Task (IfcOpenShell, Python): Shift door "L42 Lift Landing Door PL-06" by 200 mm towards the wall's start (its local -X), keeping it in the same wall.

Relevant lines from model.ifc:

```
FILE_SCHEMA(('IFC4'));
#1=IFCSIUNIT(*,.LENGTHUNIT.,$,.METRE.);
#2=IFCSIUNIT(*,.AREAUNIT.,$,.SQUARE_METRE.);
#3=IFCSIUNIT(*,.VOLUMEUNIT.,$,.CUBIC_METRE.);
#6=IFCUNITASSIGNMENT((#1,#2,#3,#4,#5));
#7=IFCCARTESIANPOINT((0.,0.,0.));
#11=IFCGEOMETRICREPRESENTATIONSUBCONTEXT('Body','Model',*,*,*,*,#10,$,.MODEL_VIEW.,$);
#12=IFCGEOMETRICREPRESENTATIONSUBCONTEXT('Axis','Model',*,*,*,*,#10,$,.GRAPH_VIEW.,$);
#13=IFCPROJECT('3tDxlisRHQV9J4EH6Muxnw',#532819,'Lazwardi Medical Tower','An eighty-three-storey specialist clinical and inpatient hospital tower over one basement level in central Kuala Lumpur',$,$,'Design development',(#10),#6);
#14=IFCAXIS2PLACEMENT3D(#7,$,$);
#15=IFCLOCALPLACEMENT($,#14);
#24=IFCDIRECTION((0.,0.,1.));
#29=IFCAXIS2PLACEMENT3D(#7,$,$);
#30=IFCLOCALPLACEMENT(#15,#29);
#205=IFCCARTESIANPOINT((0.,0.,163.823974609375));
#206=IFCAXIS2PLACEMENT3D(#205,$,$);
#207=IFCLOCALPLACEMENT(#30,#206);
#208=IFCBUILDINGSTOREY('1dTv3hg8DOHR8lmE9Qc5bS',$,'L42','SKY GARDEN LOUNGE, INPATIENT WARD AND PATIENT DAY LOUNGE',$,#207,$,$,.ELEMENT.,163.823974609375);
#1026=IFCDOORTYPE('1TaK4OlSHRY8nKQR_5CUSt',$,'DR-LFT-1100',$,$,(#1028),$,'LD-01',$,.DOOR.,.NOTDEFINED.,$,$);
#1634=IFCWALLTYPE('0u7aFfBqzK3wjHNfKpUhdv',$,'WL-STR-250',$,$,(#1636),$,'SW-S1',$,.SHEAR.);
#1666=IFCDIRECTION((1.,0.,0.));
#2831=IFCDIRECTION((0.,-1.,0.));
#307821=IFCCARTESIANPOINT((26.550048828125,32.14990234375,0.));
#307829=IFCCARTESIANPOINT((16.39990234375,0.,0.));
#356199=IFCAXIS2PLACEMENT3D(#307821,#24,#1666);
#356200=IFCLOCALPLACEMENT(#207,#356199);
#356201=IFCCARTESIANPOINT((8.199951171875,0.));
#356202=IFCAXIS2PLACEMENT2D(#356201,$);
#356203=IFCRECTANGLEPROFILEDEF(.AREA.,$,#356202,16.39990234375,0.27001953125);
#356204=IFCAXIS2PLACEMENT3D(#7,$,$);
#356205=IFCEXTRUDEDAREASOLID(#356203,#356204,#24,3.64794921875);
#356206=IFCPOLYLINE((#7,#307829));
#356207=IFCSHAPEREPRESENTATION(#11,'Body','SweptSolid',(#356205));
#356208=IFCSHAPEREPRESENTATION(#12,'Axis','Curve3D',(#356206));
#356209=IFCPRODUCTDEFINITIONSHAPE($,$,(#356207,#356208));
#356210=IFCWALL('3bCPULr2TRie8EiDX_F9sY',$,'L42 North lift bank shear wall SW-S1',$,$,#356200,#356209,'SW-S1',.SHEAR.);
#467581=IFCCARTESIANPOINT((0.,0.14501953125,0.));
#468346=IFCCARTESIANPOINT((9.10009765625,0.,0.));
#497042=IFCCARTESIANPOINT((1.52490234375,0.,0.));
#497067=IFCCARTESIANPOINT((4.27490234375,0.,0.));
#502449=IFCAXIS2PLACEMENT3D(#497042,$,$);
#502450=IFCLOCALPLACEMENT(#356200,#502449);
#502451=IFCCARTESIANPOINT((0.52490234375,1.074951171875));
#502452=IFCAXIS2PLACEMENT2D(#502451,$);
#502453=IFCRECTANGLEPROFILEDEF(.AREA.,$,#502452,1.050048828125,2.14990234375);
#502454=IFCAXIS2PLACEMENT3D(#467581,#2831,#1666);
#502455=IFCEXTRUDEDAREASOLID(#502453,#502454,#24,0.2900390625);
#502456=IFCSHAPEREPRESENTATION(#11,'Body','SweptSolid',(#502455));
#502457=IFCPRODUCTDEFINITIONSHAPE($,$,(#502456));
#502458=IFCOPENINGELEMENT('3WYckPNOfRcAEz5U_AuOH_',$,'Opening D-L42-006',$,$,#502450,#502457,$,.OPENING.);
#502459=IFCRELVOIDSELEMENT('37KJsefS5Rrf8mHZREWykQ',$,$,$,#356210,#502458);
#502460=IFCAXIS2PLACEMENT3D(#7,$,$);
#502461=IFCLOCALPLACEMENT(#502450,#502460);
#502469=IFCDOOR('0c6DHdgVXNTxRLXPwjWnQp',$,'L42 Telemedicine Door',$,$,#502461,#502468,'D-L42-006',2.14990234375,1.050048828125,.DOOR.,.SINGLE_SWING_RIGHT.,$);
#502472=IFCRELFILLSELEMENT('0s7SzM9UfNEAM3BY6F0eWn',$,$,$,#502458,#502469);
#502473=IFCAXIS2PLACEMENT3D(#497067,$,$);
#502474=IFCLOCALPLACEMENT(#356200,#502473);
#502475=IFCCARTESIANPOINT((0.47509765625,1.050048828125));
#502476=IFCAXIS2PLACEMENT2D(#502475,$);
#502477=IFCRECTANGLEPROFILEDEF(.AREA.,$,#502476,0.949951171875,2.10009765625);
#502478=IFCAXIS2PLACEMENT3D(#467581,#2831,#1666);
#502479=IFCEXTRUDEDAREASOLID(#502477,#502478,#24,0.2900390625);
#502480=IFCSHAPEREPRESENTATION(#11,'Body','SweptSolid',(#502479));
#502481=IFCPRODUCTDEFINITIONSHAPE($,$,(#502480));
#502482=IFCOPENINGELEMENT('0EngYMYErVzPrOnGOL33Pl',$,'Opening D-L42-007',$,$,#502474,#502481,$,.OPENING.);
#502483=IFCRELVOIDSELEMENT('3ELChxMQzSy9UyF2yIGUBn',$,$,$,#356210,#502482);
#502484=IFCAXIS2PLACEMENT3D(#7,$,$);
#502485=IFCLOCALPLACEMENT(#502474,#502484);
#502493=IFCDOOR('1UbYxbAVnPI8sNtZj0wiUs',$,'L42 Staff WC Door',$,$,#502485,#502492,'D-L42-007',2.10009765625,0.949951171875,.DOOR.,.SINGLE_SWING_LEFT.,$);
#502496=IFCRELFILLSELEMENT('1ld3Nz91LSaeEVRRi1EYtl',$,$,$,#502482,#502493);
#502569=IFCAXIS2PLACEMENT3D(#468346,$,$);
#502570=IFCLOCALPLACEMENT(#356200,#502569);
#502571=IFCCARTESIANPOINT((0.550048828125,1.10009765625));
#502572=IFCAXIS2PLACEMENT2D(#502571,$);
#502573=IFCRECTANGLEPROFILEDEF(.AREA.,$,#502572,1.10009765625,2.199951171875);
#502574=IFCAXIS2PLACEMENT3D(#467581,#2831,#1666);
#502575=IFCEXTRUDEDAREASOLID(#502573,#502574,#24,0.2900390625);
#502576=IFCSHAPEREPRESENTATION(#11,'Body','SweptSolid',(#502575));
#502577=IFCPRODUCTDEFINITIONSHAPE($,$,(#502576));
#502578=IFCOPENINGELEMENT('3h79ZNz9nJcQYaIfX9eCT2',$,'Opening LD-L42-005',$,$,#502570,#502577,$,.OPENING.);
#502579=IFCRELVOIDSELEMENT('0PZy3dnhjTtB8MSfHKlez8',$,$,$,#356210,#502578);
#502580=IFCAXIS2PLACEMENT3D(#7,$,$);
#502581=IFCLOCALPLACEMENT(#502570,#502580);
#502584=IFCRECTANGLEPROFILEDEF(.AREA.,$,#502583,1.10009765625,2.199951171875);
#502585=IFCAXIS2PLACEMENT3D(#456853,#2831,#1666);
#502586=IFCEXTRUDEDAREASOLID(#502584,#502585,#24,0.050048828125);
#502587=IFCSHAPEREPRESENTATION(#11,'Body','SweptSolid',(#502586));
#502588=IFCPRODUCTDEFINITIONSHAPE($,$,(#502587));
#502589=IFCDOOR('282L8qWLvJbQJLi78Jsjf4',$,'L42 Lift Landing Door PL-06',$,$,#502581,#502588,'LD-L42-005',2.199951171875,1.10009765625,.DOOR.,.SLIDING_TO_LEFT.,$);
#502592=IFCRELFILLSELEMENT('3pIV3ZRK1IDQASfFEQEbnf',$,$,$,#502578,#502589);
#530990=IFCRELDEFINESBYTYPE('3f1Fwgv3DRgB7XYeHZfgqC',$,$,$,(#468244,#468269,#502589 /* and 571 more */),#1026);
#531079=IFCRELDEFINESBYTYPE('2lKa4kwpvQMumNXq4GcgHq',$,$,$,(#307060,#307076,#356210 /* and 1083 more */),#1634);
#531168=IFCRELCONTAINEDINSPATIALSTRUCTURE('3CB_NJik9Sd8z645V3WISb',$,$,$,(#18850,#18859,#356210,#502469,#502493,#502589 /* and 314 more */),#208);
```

```python
import ifcopenshell
import ifcopenshell.api.geometry
import ifcopenshell.util.placement
import ifcopenshell.util.unit

model = ifcopenshell.open("model.ifc")
unit_scale = ifcopenshell.util.unit.calculate_unit_scale(model)

door = model.by_guid("282L8qWLvJbQJLi78Jsjf4")
opening = door.FillsVoids[0].RelatingOpeningElement
wall = opening.VoidsElements[0].RelatingBuildingElement

wall_matrix = ifcopenshell.util.placement.get_local_placement(wall.ObjectPlacement)
shift = wall_matrix[:3, 0] * -0.2 / unit_scale
before = ifcopenshell.util.placement.get_local_placement(door.ObjectPlacement)[:3, 3].copy()

# The door is placed relative to its opening, so it follows when the opening moves.
matrix = ifcopenshell.util.placement.get_local_placement(opening.ObjectPlacement)
matrix[:3, 3] += shift
ifcopenshell.api.geometry.edit_object_placement(
    model, product=opening, matrix=matrix, is_si=False, should_transform_children=True
)

after = ifcopenshell.util.placement.get_local_placement(door.ObjectPlacement)[:3, 3]
print("door moved by", (after - before).round(3) + 0.0)

model.write("model_v2.ifc")
```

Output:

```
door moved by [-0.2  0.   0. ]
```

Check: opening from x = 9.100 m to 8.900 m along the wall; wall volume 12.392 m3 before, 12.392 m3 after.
